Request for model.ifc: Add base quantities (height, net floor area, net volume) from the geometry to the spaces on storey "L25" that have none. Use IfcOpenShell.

First a look at what the model holds.

```python
import ifcopenshell
import ifcopenshell.util.element
import ifcopenshell.util.unit

model = ifcopenshell.open("model.ifc")
print(model.schema)
for unit_type in ("LENGTHUNIT", "AREAUNIT", "VOLUMEUNIT"):
    print(unit_type, ifcopenshell.util.unit.calculate_unit_scale(model, unit_type))
storey = next(s for s in model.by_type("IfcBuildingStorey") if s.Name == "L25")
spaces = [e for e in ifcopenshell.util.element.get_decomposition(storey) if e.is_a("IfcSpace")]
for e in sorted(spaces, key=lambda e: e.id()):
    print(e.id(), e.is_a(), e.Name, list(ifcopenshell.util.element.get_psets(e, qtos_only=True)), sep=" | ")
```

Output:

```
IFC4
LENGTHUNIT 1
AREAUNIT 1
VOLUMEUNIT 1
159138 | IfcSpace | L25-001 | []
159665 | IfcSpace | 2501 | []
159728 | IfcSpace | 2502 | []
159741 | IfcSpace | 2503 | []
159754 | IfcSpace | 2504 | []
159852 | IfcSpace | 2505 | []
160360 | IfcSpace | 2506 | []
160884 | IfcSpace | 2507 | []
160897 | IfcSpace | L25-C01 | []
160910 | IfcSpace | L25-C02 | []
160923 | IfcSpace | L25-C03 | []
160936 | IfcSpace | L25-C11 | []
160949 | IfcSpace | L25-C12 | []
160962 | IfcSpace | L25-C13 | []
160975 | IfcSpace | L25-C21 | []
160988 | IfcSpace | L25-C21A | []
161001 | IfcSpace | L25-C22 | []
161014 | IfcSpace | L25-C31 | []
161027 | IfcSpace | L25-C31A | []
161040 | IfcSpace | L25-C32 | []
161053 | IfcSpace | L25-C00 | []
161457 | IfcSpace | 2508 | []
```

```python
import ifcopenshell
import ifcopenshell.api.pset
import ifcopenshell.geom
import ifcopenshell.util.element
import ifcopenshell.util.shape
import ifcopenshell.util.unit

model = ifcopenshell.open("model.ifc")
unit_scale = ifcopenshell.util.unit.calculate_unit_scale(model)
area_scale = ifcopenshell.util.unit.calculate_unit_scale(model, "AREAUNIT")
volume_scale = ifcopenshell.util.unit.calculate_unit_scale(model, "VOLUMEUNIT")
settings = ifcopenshell.geom.settings()

storey = next(s for s in model.by_type("IfcBuildingStorey") if s.Name == "L25")
spaces = [e for e in ifcopenshell.util.element.get_decomposition(storey) if e.is_a("IfcSpace")]

for e in sorted(spaces, key=lambda e: e.id()):
    if ifcopenshell.util.element.get_psets(e, qtos_only=True, should_inherit=False):
        continue
    # Geometry comes back in metres, in the element's own axes.
    shape = ifcopenshell.geom.create_shape(settings, e)
    values = {
        "Height": ifcopenshell.util.shape.get_z(shape.geometry) / unit_scale,
        "NetFloorArea": ifcopenshell.util.shape.get_footprint_area(shape.geometry) / area_scale,
        "NetVolume": ifcopenshell.util.shape.get_volume(shape.geometry) / volume_scale,
    }
    qto = ifcopenshell.api.pset.add_qto(model, product=e, name="Qto_SpaceBaseQuantities")
    ifcopenshell.api.pset.edit_qto(model, qto=qto, properties=values)
    print(e.id(), {k: round(v, 3) for k, v in values.items()})

model.write("model_rev.ifc")
```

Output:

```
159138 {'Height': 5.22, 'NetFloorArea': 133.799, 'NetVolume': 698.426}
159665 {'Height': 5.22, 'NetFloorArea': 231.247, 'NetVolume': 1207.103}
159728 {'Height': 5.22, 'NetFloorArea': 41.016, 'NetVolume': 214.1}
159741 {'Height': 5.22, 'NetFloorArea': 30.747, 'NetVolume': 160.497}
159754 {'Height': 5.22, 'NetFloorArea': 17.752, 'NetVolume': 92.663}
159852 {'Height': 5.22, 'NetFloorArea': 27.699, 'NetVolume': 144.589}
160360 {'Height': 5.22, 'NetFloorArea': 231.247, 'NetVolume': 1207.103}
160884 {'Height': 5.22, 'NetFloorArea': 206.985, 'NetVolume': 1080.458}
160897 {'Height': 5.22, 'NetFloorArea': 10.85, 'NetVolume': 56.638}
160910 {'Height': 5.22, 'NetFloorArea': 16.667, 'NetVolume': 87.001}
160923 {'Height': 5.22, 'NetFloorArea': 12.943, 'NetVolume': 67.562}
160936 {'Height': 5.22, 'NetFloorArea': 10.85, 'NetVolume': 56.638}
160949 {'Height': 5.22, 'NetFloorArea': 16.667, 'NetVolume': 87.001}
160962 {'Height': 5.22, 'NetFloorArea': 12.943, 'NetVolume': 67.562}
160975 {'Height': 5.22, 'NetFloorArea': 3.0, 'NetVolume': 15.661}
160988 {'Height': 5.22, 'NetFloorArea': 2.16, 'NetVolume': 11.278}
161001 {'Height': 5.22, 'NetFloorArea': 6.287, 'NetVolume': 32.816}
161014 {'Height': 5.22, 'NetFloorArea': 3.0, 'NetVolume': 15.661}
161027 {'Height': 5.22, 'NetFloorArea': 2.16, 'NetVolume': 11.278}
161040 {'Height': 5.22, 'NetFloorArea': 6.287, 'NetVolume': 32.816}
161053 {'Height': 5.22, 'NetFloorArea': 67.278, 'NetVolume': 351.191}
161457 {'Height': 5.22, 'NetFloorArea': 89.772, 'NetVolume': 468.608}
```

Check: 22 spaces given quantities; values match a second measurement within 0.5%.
